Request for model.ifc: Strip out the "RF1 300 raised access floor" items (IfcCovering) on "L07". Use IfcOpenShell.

First a look at what the model holds.

```python
import ifcopenshell
import ifcopenshell.util.element

model = ifcopenshell.open("model.ifc")
print(model.schema)
storey = next(s for s in model.by_type("IfcBuildingStorey") if s.Name == "L07")
coverings = [e for e in ifcopenshell.util.element.get_decomposition(storey) if e.is_a("IfcCovering")]
seen = {}
for e in coverings:
    element_type = ifcopenshell.util.element.get_type(e)
    name = element_type.Name if element_type not in (None, e) else None
    seen[name] = seen.get(name, 0) + 1
for name, count in sorted(seen.items(), key=str):
    print(count, "x", name)
```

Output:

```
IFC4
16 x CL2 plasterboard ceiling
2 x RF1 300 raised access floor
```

```python
import ifcopenshell
import ifcopenshell.api.root
import ifcopenshell.util.element

model = ifcopenshell.open("model.ifc")

storey = next(s for s in model.by_type("IfcBuildingStorey") if s.Name == "L07")
coverings = [e for e in ifcopenshell.util.element.get_decomposition(storey) if e.is_a("IfcCovering")]
targets = [e for e in coverings if (t := ifcopenshell.util.element.get_type(e)) not in (None, e) and t.Name == "RF1 300 raised access floor"]

for e in targets:
    ifcopenshell.api.root.remove_product(model, product=e)
print(len(targets), "removed")

model.write("model_rev.ifc")
```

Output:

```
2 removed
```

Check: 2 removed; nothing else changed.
